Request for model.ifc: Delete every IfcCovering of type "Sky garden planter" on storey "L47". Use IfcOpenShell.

First a look at what the model holds.

```python
import ifcopenshell
import ifcopenshell.util.element

model = ifcopenshell.open("model.ifc")
print(model.schema)
storey = next(s for s in model.by_type("IfcBuildingStorey") if s.Name == "L47")
coverings = [e for e in ifcopenshell.util.element.get_decomposition(storey) if e.is_a("IfcCovering")]
seen = {}
for e in coverings:
    element_type = ifcopenshell.util.element.get_type(e)
    name = element_type.Name if element_type not in (None, e) else None
    seen[name] = seen.get(name, 0) + 1
for name, count in sorted(seen.items(), key=str):
    print(count, "x", name)
```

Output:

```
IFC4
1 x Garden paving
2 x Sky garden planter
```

```python
import ifcopenshell
import ifcopenshell.api.root
import ifcopenshell.util.element

model = ifcopenshell.open("model.ifc")

storey = next(s for s in model.by_type("IfcBuildingStorey") if s.Name == "L47")
coverings = [e for e in ifcopenshell.util.element.get_decomposition(storey) if e.is_a("IfcCovering")]
targets = [e for e in coverings if (t := ifcopenshell.util.element.get_type(e)) not in (None, e) and t.Name == "Sky garden planter"]

for e in targets:
    ifcopenshell.api.root.remove_product(model, product=e)
print(len(targets), "removed")

model.write("model_v2.ifc")
```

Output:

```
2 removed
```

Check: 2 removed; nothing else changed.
